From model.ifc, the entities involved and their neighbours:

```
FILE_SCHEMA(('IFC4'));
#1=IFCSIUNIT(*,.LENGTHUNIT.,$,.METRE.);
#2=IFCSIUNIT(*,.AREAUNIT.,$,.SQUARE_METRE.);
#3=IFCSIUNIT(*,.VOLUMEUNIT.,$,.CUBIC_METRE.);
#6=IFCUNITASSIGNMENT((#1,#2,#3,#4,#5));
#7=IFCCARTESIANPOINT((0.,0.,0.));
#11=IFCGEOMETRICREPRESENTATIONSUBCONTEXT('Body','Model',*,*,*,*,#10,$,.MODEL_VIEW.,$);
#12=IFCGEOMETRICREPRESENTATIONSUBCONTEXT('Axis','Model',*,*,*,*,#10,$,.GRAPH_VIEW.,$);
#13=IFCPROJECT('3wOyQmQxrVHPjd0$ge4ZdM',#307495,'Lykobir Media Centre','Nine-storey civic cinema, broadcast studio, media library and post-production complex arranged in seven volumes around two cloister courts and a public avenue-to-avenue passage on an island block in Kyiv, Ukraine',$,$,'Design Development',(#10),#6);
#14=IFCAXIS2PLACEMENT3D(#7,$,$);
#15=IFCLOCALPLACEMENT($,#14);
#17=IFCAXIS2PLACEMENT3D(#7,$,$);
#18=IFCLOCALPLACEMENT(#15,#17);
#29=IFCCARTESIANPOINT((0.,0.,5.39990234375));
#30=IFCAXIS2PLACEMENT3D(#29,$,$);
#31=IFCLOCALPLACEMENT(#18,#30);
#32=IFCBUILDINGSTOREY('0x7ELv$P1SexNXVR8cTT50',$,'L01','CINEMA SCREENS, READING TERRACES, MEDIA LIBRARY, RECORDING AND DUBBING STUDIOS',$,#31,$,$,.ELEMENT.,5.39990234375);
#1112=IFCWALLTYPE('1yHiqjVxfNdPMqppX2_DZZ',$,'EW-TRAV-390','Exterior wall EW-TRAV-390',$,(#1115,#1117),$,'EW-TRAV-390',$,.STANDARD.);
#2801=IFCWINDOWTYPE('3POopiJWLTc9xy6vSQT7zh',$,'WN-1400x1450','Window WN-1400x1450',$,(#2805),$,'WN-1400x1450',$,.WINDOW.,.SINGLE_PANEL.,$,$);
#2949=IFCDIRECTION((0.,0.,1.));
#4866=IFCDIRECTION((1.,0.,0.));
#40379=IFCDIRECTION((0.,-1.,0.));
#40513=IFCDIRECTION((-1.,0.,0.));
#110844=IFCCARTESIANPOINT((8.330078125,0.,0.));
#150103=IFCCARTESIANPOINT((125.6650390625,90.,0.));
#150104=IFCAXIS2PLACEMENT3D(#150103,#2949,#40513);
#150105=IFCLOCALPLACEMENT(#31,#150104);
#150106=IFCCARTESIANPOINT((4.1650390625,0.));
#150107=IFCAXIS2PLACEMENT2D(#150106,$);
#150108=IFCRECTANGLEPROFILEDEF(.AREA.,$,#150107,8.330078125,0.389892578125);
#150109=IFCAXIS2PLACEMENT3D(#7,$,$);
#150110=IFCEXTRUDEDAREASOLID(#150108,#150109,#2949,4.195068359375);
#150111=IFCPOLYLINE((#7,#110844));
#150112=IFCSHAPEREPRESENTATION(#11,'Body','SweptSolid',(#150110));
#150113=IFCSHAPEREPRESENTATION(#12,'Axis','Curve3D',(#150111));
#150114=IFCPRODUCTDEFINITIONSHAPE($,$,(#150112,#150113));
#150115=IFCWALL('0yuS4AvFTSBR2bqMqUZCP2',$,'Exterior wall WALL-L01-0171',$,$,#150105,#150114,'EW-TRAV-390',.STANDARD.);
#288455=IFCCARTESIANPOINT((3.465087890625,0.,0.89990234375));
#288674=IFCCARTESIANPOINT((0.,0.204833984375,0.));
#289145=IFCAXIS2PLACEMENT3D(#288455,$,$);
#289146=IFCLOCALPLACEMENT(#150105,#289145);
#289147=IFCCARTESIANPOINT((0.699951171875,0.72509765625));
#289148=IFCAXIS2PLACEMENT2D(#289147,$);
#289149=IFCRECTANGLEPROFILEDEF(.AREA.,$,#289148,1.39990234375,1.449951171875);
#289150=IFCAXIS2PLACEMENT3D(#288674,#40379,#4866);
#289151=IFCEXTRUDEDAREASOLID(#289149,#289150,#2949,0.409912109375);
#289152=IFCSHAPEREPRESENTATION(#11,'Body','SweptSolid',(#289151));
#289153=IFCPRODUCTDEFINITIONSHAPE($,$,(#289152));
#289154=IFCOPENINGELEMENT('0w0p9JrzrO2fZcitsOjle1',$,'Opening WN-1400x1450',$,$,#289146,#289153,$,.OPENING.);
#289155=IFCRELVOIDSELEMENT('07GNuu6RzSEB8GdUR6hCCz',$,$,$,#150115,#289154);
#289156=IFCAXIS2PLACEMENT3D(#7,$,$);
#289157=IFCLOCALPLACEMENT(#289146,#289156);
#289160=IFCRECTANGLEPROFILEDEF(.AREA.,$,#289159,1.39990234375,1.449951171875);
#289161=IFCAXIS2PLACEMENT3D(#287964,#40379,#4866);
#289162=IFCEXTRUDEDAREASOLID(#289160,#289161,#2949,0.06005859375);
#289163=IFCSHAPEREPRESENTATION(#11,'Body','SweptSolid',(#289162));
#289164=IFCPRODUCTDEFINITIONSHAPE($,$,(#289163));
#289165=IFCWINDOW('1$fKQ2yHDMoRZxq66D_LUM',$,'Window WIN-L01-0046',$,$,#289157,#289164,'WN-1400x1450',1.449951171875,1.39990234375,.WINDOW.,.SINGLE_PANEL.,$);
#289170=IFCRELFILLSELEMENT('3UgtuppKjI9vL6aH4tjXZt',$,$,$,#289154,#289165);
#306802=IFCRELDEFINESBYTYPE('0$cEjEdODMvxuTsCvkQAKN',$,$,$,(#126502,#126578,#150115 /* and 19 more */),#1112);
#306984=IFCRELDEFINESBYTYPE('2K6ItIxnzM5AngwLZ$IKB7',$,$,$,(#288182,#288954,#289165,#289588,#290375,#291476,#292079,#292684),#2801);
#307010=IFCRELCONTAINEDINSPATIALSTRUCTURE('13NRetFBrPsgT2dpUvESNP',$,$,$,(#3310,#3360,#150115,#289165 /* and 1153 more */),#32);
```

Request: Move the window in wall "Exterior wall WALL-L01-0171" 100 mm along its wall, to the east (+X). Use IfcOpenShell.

```python
import ifcopenshell
import ifcopenshell.api.geometry
import ifcopenshell.util.placement

model = ifcopenshell.open("model.ifc")

window = model.by_guid("1$fKQ2yHDMoRZxq66D_LUM")
opening = window.FillsVoids[0].RelatingOpeningElement
wall = opening.VoidsElements[0].RelatingBuildingElement

wall_matrix = ifcopenshell.util.placement.get_local_placement(wall.ObjectPlacement)
shift = wall_matrix[:3, 0] * -0.1
before = ifcopenshell.util.placement.get_local_placement(window.ObjectPlacement)[:3, 3].copy()

# The window is placed relative to its opening, so it follows when the opening moves.
matrix = ifcopenshell.util.placement.get_local_placement(opening.ObjectPlacement)
matrix[:3, 3] += shift
ifcopenshell.api.geometry.edit_object_placement(
    model, product=opening, matrix=matrix, is_si=False, should_transform_children=True
)

after = ifcopenshell.util.placement.get_local_placement(window.ObjectPlacement)[:3, 3]
print("window moved by", (after - before).round(3) + 0.0)

model.write("model-out.ifc")
```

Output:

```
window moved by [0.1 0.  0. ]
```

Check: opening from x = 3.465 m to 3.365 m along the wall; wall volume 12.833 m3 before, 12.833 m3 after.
